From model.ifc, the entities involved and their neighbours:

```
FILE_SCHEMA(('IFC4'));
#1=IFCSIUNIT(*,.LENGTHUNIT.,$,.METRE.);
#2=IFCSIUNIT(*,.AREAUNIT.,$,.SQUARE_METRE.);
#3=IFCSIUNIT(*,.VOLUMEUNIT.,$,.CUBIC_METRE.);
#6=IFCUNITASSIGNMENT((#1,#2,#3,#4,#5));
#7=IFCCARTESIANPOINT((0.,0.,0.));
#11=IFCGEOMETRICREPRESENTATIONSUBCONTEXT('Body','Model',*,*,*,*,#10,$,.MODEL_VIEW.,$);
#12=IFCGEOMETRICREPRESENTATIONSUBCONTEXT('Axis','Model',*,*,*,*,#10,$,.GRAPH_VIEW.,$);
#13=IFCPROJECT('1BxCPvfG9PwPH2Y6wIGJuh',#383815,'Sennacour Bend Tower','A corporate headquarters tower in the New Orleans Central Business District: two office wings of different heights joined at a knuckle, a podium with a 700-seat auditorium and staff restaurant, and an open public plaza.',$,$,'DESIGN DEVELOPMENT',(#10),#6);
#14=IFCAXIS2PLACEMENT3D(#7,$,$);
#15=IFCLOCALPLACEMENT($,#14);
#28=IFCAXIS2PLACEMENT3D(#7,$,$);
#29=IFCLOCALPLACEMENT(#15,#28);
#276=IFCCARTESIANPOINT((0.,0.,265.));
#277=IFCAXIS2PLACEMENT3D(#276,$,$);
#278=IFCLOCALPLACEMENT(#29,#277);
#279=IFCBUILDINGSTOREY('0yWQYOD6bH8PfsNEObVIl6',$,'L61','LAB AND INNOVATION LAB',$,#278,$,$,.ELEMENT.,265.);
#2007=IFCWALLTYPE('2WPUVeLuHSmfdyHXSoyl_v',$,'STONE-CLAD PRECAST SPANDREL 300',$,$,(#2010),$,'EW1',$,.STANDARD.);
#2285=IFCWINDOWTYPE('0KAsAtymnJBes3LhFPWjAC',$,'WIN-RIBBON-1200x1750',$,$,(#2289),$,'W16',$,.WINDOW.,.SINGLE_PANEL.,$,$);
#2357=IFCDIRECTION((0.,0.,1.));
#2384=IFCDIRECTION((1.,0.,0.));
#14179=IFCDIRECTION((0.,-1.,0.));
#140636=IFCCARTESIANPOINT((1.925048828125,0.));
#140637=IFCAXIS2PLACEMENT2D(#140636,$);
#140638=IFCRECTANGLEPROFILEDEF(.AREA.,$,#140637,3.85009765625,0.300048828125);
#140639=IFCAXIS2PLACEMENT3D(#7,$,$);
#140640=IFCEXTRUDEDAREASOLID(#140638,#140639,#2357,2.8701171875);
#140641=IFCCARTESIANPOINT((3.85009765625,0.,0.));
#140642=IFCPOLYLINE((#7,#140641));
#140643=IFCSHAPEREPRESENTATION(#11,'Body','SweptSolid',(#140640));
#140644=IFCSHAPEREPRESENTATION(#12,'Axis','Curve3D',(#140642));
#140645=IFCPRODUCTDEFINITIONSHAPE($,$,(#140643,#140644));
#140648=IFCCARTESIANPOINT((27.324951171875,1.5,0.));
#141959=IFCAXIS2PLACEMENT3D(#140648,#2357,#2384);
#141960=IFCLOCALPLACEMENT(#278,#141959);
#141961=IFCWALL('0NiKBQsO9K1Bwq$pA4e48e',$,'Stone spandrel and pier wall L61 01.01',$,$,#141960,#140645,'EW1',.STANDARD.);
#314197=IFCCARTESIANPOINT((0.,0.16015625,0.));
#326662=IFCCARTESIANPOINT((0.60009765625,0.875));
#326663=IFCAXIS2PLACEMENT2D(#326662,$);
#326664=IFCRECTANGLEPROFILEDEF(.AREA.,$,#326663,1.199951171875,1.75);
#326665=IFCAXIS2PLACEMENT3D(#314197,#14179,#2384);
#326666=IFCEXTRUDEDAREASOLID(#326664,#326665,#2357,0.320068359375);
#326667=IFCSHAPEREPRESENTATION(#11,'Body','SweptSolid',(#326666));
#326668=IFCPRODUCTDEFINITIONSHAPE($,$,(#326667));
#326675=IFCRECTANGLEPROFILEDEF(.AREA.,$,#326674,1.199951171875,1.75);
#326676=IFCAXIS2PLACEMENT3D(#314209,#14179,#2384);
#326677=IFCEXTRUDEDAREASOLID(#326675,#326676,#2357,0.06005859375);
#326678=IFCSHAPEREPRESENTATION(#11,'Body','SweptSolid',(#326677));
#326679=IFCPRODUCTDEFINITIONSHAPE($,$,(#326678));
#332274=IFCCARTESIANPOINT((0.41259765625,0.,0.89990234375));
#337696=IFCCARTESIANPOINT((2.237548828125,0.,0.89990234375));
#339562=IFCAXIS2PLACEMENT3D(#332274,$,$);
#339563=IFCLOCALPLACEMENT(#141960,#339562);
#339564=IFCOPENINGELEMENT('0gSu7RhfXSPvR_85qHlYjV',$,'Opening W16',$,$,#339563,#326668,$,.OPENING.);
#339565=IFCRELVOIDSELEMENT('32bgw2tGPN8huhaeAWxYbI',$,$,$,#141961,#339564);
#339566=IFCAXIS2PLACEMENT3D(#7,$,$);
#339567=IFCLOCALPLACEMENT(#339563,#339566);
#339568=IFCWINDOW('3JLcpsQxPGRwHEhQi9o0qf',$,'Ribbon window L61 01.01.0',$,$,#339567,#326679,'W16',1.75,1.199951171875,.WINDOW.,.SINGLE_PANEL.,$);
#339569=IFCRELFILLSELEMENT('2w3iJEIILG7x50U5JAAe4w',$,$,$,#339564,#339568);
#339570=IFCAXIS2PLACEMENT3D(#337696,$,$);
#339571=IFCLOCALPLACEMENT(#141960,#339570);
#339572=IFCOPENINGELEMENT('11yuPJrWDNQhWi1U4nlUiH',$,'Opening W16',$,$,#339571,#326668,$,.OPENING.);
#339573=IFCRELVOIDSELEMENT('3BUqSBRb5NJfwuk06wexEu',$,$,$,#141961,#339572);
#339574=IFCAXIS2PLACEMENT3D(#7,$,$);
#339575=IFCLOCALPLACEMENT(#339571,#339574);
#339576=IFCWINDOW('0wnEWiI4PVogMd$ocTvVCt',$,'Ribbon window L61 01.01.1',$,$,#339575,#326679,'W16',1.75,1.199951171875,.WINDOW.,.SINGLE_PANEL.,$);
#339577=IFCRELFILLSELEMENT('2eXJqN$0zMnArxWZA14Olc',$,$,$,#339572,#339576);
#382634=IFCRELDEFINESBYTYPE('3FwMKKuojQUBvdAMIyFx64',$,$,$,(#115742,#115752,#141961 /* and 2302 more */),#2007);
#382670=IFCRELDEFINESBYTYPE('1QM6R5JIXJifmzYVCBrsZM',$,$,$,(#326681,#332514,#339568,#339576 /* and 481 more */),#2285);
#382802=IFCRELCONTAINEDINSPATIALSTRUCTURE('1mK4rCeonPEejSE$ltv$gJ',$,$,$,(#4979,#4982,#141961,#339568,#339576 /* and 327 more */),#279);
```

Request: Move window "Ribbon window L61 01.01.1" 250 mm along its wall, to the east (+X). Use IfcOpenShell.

```python
import ifcopenshell
import ifcopenshell.api.geometry
import ifcopenshell.util.placement
import ifcopenshell.util.unit

model = ifcopenshell.open("model.ifc")
unit_scale = ifcopenshell.util.unit.calculate_unit_scale(model)

window = model.by_guid("0wnEWiI4PVogMd$ocTvVCt")
opening = window.FillsVoids[0].RelatingOpeningElement
wall = opening.VoidsElements[0].RelatingBuildingElement

wall_matrix = ifcopenshell.util.placement.get_local_placement(wall.ObjectPlacement)
shift = wall_matrix[:3, 0] * 0.25 / unit_scale
before = ifcopenshell.util.placement.get_local_placement(window.ObjectPlacement)[:3, 3].copy()

# The window is placed relative to its opening, so it follows when the opening moves.
matrix = ifcopenshell.util.placement.get_local_placement(opening.ObjectPlacement)
matrix[:3, 3] += shift
ifcopenshell.api.geometry.edit_object_placement(
    model, product=opening, matrix=matrix, is_si=False, should_transform_children=True
)

after = ifcopenshell.util.placement.get_local_placement(window.ObjectPlacement)[:3, 3]
print("window moved by", (after - before).round(3) + 0.0)

model.write("model_v2.ifc")
```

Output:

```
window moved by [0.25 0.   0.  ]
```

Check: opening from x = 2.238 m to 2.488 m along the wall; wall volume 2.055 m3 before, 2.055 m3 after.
